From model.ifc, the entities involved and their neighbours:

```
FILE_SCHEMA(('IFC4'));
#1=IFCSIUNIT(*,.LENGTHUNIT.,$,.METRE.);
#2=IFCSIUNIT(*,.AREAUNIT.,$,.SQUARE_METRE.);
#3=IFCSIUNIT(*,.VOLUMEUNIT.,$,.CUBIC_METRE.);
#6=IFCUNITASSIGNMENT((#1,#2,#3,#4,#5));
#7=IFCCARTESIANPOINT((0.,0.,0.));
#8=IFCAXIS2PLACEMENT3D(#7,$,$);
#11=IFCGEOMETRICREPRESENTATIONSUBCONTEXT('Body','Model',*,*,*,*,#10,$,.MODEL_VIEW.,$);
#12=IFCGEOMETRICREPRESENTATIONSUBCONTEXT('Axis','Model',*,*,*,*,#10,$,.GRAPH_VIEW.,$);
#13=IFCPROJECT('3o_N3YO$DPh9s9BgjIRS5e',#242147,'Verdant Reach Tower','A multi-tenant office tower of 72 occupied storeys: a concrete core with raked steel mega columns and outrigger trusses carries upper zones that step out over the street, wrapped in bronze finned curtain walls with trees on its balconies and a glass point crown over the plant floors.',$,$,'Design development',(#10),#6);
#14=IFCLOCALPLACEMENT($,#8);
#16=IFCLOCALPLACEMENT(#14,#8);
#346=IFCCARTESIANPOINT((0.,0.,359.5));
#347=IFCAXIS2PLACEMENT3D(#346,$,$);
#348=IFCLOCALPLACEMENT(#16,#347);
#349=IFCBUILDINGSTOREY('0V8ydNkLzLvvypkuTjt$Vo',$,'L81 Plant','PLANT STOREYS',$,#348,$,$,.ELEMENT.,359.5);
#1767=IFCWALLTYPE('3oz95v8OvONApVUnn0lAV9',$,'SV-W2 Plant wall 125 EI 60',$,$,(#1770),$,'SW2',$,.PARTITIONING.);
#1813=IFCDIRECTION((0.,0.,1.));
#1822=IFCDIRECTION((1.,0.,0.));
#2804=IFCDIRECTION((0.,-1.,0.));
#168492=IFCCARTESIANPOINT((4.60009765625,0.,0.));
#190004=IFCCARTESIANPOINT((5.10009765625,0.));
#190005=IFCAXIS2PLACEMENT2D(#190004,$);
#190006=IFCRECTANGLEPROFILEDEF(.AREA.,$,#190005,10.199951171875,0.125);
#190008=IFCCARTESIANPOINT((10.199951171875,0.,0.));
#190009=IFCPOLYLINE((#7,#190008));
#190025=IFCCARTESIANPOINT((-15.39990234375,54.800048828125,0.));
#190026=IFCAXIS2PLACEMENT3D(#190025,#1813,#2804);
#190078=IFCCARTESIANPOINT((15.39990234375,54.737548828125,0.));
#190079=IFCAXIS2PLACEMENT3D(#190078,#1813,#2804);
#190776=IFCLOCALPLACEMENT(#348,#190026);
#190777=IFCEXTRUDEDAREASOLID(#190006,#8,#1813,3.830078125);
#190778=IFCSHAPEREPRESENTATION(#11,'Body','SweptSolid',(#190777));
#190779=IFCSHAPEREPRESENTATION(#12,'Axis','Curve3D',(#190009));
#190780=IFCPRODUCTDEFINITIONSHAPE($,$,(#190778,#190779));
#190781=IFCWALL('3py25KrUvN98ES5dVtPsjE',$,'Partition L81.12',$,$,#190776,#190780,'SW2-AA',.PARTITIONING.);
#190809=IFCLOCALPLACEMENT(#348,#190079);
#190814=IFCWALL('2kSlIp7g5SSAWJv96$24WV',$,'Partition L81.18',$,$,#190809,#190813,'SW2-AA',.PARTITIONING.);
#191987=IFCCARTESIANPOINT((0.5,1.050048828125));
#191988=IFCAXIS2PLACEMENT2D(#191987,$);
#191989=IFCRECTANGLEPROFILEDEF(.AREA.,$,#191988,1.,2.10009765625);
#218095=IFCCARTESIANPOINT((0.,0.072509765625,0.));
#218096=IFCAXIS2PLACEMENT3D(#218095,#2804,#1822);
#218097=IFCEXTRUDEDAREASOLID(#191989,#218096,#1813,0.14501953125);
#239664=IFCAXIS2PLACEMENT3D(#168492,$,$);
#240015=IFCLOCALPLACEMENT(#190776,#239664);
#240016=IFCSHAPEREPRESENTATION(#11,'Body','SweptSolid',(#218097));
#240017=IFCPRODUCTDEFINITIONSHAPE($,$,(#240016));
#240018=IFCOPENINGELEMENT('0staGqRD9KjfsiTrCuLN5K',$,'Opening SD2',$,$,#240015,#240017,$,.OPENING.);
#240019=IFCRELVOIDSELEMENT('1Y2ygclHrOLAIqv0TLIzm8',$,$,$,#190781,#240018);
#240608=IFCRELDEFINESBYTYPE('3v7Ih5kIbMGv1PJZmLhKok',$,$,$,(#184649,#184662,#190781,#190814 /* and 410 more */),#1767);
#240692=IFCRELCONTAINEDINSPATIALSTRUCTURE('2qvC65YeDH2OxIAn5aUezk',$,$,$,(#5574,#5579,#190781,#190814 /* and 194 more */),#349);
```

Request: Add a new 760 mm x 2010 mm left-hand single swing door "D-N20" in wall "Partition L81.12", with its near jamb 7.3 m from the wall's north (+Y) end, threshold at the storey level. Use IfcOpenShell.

```python
import numpy as np
import ifcopenshell
import ifcopenshell.api.feature
import ifcopenshell.api.geometry
import ifcopenshell.api.root
import ifcopenshell.api.spatial
import ifcopenshell.geom
import ifcopenshell.util.element
import ifcopenshell.util.placement
import ifcopenshell.util.representation
import ifcopenshell.util.shape
import ifcopenshell.util.unit

model = ifcopenshell.open("model.ifc")
unit_scale = ifcopenshell.util.unit.calculate_unit_scale(model)
settings = ifcopenshell.geom.settings()


def volume(element):
    """Net volume in cubic metres, openings subtracted."""
    shape = ifcopenshell.geom.create_shape(settings, element)
    return ifcopenshell.util.shape.get_volume(shape.geometry)


wall = model.by_guid("3py25KrUvN98ES5dVtPsjE")
storey = ifcopenshell.util.element.get_container(wall, ifc_class="IfcBuildingStorey")
context = ifcopenshell.util.representation.get_context(model, "Model", "Body", "MODEL_VIEW")
before = volume(wall)

width, height, from_end, sill = 0.76, 2.01, 7.3, 0.0  # metres

# The wall runs along its own X axis, and the end named is its -X end.
wall_shape = ifcopenshell.geom.create_shape(settings, wall)
x, y, z = ifcopenshell.util.shape.get_vertices(wall_shape.geometry).T
start = x.min() + from_end
face, thickness = float(y.min()), float(y.max() - y.min())
wall_matrix = ifcopenshell.util.placement.get_local_placement(wall.ObjectPlacement)
level = ifcopenshell.util.placement.get_local_placement(storey.ObjectPlacement)[2, 3]


def in_wall(x, y):
    """Placement at x, y metres in the wall's axes, at sill height."""
    matrix = wall_matrix.copy()
    matrix[:, 3] = wall_matrix @ np.array([x / unit_scale, y / unit_scale, 0.0, 1.0])
    matrix[2, 3] = level + sill / unit_scale
    return matrix


# Opening: a box that overshoots both wall faces by 50 mm.
opening = ifcopenshell.api.root.create_entity(model, ifc_class="IfcOpeningElement", predefined_type="OPENING")
box = ifcopenshell.api.geometry.add_wall_representation(
    model, context=context, length=width, height=height, thickness=thickness + 0.1
)
ifcopenshell.api.geometry.assign_representation(model, product=opening, representation=box)
ifcopenshell.api.geometry.edit_object_placement(model, product=opening, matrix=in_wall(start, face - 0.05), is_si=False)
ifcopenshell.api.feature.add_feature(model, feature=opening, element=wall)

door = ifcopenshell.api.root.create_entity(model, ifc_class="IfcDoor", name="D-N20", predefined_type="DOOR")
door.OverallWidth, door.OverallHeight = width / unit_scale, height / unit_scale
door.OperationType = "SINGLE_SWING_LEFT"
body = ifcopenshell.api.geometry.add_door_representation(
    model,
    context=context,
    overall_width=door.OverallWidth,
    overall_height=door.OverallHeight,
    operation_type="SINGLE_SWING_LEFT",
    lining_properties={"LiningDepth": thickness / unit_scale, "ThresholdDepth": thickness / unit_scale},
)
ifcopenshell.api.geometry.assign_representation(model, product=door, representation=body)
ifcopenshell.api.spatial.assign_container(model, products=[door], relating_structure=storey)
ifcopenshell.api.feature.add_filling(model, opening=opening, element=door)

# The lining spans the wall, so the door starts at the wall face.
ifcopenshell.api.geometry.edit_object_placement(model, product=door, matrix=in_wall(start, face), is_si=False)

after = volume(wall)

print(f"wall volume {before:.3f} -> {after:.3f} m3")

model.write("model_edited.ifc")
```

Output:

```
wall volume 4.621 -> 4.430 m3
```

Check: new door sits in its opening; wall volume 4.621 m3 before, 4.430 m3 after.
